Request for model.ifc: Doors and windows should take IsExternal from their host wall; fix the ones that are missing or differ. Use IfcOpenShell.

First a look at what the model holds.

```python
import ifcopenshell
import ifcopenshell.util.element

model = ifcopenshell.open("model.ifc")
print(model.schema)
seen = {}
for e in model.by_type("IfcDoor") + model.by_type("IfcWindow"):
    if not e.FillsVoids:
        continue
    host = e.FillsVoids[0].RelatingOpeningElement.VoidsElements[0].RelatingBuildingElement
    own = ifcopenshell.util.element.get_pset(e, f"Pset_{e.is_a()[3:].removesuffix('StandardCase')}Common", "IsExternal")
    wall = ifcopenshell.util.element.get_pset(host, "Pset_WallCommon", "IsExternal")
    seen[e.is_a(), own, wall] = seen.get((e.is_a(), own, wall), 0) + 1
for (cls, own, wall), count in sorted(seen.items(), key=str):
    print(count, cls, "IsExternal:", own, "| host wall:", wall)
```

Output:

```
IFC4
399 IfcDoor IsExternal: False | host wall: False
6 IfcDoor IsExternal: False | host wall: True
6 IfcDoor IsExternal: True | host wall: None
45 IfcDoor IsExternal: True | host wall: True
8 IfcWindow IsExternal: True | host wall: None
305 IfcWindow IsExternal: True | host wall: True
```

```python
import ifcopenshell
import ifcopenshell.api.pset
import ifcopenshell.util.element

model = ifcopenshell.open("model.ifc")

count = 0
for ifc_class, pset_name in (("IfcDoor", "Pset_DoorCommon"), ("IfcWindow", "Pset_WindowCommon")):
    for e in model.by_type(ifc_class):
        if not e.FillsVoids:
            continue
        host = e.FillsVoids[0].RelatingOpeningElement.VoidsElements[0].RelatingBuildingElement
        external = ifcopenshell.util.element.get_pset(host, "Pset_WallCommon", "IsExternal")
        if external is None or ifcopenshell.util.element.get_pset(e, pset_name, "IsExternal") == external:
            continue
        pset = ifcopenshell.api.pset.add_pset(model, product=e, name=pset_name)
        ifcopenshell.api.pset.edit_pset(model, pset=pset, properties={"IsExternal": external})
        count += 1

print(count, "updated")

model.write("model-out.ifc")
```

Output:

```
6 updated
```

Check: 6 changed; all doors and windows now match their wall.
